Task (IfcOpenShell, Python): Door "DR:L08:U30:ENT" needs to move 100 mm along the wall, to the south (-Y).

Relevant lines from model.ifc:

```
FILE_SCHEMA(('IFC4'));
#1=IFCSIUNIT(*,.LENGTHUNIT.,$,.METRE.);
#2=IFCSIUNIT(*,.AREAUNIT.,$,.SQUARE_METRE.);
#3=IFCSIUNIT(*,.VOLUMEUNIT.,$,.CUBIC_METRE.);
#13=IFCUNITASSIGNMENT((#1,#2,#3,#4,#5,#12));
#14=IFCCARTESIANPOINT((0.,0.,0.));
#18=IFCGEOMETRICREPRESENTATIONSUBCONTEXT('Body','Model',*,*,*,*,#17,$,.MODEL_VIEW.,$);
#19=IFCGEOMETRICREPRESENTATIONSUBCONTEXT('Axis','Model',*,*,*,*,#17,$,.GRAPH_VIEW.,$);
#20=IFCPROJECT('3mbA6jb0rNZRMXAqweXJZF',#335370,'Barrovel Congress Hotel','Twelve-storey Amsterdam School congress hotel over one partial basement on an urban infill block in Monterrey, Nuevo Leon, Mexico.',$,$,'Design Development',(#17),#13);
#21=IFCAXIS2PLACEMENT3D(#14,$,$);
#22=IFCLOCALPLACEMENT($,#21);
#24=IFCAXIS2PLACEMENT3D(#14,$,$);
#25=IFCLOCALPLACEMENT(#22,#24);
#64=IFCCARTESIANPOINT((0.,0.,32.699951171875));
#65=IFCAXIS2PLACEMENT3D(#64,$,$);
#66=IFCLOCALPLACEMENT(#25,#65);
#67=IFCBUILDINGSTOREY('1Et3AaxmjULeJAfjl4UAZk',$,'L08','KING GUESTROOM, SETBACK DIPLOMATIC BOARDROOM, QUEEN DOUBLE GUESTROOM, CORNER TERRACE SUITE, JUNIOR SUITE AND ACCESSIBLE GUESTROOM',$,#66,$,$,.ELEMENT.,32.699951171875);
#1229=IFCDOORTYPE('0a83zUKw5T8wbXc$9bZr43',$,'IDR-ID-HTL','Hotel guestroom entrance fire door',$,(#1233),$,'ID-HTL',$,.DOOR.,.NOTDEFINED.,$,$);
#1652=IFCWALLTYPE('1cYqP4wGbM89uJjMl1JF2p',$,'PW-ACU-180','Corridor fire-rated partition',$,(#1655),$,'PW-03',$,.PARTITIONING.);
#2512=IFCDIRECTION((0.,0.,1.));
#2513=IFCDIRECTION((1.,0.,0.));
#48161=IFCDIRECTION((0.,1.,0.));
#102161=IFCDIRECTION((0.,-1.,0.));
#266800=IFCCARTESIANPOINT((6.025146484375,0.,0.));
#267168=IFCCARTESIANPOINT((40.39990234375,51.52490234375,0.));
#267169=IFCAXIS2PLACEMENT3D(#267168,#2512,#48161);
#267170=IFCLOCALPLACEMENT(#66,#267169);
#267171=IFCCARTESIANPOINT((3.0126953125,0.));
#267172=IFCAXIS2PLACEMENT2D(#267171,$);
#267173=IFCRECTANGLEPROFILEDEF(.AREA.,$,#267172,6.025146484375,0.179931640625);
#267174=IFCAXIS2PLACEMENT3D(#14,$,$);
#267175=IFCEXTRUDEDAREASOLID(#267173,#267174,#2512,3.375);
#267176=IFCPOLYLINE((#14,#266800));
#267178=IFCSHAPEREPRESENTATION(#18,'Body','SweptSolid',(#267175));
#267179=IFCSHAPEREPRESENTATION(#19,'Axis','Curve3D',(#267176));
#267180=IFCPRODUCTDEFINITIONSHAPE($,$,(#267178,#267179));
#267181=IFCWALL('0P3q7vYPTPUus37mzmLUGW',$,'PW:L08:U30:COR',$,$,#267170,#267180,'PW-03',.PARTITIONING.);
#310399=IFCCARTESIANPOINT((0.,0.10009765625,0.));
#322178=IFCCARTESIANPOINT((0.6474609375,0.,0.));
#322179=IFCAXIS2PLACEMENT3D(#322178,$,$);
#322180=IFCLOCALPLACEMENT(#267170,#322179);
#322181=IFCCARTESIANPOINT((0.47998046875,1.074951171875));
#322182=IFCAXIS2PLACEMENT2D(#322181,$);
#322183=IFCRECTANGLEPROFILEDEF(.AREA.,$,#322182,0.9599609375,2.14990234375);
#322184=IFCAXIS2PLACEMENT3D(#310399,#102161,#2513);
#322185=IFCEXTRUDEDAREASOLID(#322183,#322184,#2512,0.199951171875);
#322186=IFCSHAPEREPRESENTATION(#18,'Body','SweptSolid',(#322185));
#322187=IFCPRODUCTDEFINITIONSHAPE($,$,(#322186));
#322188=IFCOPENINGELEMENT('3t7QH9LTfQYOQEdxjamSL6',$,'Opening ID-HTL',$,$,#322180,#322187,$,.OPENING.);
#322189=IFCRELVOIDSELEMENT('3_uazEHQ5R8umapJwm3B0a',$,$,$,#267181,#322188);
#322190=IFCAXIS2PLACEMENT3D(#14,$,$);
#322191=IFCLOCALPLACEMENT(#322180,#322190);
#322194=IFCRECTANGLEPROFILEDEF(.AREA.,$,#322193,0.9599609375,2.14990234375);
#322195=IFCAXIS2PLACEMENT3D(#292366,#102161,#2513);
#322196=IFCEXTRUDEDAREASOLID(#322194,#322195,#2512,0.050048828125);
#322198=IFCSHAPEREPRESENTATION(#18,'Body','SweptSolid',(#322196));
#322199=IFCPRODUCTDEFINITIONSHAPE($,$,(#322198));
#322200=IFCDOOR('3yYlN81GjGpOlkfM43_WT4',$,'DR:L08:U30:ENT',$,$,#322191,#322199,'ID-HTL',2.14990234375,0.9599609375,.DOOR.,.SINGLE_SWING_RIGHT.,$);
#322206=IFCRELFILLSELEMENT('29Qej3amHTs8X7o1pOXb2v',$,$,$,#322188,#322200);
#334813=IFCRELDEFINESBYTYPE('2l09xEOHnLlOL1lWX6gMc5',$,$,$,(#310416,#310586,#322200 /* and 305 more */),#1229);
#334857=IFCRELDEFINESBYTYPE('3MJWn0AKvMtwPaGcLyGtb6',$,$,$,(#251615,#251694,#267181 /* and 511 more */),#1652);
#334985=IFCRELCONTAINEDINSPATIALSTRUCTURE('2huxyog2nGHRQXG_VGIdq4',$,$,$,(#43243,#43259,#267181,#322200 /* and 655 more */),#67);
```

```python
import ifcopenshell
import ifcopenshell.api.geometry
import ifcopenshell.util.placement
import ifcopenshell.util.unit

model = ifcopenshell.open("model.ifc")
unit_scale = ifcopenshell.util.unit.calculate_unit_scale(model)

door = model.by_guid("3yYlN81GjGpOlkfM43_WT4")
opening = door.FillsVoids[0].RelatingOpeningElement
wall = opening.VoidsElements[0].RelatingBuildingElement

wall_matrix = ifcopenshell.util.placement.get_local_placement(wall.ObjectPlacement)
shift = wall_matrix[:3, 0] * -0.1 / unit_scale
before = ifcopenshell.util.placement.get_local_placement(door.ObjectPlacement)[:3, 3].copy()

# The door is placed relative to its opening, so it follows when the opening moves.
matrix = ifcopenshell.util.placement.get_local_placement(opening.ObjectPlacement)
matrix[:3, 3] += shift
ifcopenshell.api.geometry.edit_object_placement(
    model, product=opening, matrix=matrix, is_si=False, should_transform_children=True
)

after = ifcopenshell.util.placement.get_local_placement(door.ObjectPlacement)[:3, 3]
print("door moved by", (after - before).round(3) + 0.0)

model.write("model_rev.ifc")
```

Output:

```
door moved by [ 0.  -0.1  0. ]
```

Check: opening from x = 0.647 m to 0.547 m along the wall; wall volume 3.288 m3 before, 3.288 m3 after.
